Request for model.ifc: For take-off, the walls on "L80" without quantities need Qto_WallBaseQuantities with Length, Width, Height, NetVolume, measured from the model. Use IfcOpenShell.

First a look at what the model holds.

```python
import ifcopenshell
import ifcopenshell.util.element
import ifcopenshell.util.unit

model = ifcopenshell.open("model.ifc")
print(model.schema)
for unit_type in ("LENGTHUNIT", "AREAUNIT", "VOLUMEUNIT"):
    print(unit_type, ifcopenshell.util.unit.calculate_unit_scale(model, unit_type))
storey = next(s for s in model.by_type("IfcBuildingStorey") if s.Name == "L80")
walls = [e for e in ifcopenshell.util.element.get_decomposition(storey) if e.is_a("IfcWall")]
for e in sorted(walls, key=lambda e: e.id()):
    print(e.id(), e.is_a(), e.Name, list(ifcopenshell.util.element.get_psets(e, qtos_only=True)), sep=" | ")
```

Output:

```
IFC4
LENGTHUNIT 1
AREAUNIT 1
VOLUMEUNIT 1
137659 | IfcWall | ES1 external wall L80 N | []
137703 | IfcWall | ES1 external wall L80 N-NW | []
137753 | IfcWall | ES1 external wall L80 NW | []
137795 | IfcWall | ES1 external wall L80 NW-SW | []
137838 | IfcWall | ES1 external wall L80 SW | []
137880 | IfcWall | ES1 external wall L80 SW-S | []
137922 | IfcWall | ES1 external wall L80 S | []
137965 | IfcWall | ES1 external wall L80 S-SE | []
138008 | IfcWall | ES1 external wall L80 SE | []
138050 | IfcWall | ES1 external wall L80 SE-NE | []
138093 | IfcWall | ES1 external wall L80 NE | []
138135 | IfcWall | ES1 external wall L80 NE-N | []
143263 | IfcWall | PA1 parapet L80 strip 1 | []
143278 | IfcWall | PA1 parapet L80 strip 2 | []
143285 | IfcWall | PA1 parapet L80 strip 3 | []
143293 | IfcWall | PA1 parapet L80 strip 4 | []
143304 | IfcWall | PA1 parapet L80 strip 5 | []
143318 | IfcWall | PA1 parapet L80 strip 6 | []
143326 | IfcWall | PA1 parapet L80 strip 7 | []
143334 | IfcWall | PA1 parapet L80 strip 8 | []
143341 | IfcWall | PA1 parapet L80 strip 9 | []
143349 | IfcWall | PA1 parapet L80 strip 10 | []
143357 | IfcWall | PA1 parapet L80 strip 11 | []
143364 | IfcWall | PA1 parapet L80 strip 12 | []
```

```python
import ifcopenshell
import ifcopenshell.api.pset
import ifcopenshell.geom
import ifcopenshell.util.element
import ifcopenshell.util.shape
import ifcopenshell.util.unit

model = ifcopenshell.open("model.ifc")
unit_scale = ifcopenshell.util.unit.calculate_unit_scale(model)
volume_scale = ifcopenshell.util.unit.calculate_unit_scale(model, "VOLUMEUNIT")
settings = ifcopenshell.geom.settings()

storey = next(s for s in model.by_type("IfcBuildingStorey") if s.Name == "L80")
walls = [e for e in ifcopenshell.util.element.get_decomposition(storey) if e.is_a("IfcWall")]

for e in sorted(walls, key=lambda e: e.id()):
    if ifcopenshell.util.element.get_psets(e, qtos_only=True, should_inherit=False):
        continue
    # Geometry comes back in metres, in the element's own axes.
    shape = ifcopenshell.geom.create_shape(settings, e)
    values = {
        "Length": ifcopenshell.util.shape.get_x(shape.geometry) / unit_scale,
        "Width": ifcopenshell.util.shape.get_y(shape.geometry) / unit_scale,
        "Height": ifcopenshell.util.shape.get_z(shape.geometry) / unit_scale,
        "NetVolume": ifcopenshell.util.shape.get_volume(shape.geometry) / volume_scale,
    }
    qto = ifcopenshell.api.pset.add_qto(model, product=e, name="Qto_WallBaseQuantities")
    ifcopenshell.api.pset.edit_qto(model, qto=qto, properties=values)
    print(e.id(), {k: round(v, 3) for k, v in values.items()})

model.write("model_v2.ifc")
```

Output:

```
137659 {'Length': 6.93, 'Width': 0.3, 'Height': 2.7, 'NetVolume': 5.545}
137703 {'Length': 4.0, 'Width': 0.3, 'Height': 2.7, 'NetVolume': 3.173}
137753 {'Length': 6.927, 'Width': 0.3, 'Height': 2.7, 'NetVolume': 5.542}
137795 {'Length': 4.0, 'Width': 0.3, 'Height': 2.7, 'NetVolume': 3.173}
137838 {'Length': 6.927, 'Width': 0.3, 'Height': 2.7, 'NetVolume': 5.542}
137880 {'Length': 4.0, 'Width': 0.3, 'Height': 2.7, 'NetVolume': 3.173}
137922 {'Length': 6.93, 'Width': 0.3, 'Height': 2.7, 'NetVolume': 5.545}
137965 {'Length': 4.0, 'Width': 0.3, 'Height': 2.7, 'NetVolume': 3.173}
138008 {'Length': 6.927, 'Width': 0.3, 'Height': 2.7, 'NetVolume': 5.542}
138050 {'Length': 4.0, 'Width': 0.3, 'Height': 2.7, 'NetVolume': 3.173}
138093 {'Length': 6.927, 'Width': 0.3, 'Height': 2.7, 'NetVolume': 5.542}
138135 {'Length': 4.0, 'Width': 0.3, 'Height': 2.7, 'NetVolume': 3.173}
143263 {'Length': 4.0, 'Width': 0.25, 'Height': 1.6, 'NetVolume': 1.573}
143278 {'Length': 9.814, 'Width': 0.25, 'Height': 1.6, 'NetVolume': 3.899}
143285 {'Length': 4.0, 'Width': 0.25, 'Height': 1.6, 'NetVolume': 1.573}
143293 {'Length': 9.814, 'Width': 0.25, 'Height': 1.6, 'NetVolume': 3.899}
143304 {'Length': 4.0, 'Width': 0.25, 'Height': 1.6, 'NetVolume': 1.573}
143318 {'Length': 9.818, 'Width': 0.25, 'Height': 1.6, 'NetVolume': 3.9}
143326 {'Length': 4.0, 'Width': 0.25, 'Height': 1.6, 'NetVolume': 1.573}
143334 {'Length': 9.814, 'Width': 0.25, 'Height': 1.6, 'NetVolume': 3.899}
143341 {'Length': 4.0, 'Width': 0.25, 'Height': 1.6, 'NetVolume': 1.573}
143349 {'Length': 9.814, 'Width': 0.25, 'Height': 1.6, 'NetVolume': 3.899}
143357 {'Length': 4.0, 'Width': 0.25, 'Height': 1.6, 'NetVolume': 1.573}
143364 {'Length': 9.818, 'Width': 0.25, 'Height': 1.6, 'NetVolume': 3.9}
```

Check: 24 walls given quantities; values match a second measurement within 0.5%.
